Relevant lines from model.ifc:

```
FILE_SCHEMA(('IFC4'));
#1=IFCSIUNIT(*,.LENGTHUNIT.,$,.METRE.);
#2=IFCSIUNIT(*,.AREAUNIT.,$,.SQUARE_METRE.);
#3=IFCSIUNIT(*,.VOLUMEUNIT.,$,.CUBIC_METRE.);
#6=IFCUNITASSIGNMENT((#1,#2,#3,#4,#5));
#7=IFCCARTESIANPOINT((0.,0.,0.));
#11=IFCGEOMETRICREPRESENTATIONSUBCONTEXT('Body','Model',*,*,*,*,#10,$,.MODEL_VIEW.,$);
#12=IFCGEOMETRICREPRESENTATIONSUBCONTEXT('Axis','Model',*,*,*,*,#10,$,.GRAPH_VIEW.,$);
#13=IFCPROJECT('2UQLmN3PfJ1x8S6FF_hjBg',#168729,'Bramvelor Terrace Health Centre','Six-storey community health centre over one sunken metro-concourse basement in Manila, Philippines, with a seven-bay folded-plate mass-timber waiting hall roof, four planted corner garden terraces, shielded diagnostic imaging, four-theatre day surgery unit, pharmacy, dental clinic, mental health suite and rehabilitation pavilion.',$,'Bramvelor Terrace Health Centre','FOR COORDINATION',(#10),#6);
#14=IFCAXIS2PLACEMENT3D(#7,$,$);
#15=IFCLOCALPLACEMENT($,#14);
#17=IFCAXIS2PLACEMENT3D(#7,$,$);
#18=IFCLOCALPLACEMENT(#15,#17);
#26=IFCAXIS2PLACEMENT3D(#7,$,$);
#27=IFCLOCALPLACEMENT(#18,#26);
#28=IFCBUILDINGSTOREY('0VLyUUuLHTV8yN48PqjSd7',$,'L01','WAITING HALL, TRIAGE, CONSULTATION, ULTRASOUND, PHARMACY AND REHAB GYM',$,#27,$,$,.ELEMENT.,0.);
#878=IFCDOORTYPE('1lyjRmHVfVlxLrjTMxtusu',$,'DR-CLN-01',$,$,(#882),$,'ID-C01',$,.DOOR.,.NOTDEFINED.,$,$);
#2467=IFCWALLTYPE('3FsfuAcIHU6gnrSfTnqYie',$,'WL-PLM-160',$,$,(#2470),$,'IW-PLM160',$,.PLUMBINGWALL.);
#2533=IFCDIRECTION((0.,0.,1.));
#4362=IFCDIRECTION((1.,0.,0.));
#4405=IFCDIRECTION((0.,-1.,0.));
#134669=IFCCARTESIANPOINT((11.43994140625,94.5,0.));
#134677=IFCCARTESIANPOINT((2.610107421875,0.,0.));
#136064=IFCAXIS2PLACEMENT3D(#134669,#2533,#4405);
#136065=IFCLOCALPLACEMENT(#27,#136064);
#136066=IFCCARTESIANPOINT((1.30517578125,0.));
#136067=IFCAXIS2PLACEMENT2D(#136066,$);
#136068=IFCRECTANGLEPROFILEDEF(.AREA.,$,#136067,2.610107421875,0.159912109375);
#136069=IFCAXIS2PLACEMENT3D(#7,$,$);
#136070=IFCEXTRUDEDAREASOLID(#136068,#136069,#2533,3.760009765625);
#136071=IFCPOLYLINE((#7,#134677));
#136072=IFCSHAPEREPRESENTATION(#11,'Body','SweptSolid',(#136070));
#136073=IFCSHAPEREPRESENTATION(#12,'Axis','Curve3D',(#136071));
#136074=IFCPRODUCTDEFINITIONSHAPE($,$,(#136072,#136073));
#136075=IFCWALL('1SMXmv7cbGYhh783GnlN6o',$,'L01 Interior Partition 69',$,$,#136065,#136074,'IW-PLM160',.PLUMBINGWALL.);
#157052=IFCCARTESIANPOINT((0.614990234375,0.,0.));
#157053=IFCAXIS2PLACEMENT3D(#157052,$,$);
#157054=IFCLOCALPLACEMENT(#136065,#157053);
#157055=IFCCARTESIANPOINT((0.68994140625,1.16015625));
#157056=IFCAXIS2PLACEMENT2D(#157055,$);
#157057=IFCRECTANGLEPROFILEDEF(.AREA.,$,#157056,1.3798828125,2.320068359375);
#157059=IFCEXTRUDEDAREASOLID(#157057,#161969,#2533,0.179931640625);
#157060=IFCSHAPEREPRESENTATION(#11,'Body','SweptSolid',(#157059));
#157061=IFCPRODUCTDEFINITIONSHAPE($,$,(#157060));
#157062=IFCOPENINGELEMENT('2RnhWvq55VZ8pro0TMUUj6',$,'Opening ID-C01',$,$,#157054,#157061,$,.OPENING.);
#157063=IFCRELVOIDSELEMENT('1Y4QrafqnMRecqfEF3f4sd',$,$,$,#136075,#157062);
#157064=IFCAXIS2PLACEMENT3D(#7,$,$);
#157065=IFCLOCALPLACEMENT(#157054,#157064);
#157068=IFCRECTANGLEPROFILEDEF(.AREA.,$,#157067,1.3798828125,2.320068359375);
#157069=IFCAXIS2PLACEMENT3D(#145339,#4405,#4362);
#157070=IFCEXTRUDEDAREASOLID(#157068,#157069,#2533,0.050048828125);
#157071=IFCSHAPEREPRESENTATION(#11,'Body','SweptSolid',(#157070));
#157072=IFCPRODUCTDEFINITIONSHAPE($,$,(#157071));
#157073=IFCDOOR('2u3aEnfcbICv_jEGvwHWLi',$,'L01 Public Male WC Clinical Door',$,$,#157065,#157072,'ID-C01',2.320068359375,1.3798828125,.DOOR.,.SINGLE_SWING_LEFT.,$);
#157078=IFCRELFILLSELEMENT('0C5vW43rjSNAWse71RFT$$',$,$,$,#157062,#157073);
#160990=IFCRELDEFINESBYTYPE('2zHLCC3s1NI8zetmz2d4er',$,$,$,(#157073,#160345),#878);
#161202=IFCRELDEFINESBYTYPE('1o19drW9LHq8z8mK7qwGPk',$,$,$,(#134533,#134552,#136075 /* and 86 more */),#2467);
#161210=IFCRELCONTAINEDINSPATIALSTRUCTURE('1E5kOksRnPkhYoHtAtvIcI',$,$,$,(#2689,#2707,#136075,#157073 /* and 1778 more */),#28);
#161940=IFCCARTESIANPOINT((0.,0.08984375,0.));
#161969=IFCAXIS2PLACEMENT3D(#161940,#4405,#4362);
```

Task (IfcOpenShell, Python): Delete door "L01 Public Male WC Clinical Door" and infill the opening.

```python
import ifcopenshell
import ifcopenshell.api.feature
import ifcopenshell.api.root
import ifcopenshell.geom
import ifcopenshell.util.shape

model = ifcopenshell.open("model.ifc")
settings = ifcopenshell.geom.settings()


def volume(element):
    """Net volume in cubic metres, openings subtracted."""
    shape = ifcopenshell.geom.create_shape(settings, element)
    return ifcopenshell.util.shape.get_volume(shape.geometry)


door = model.by_guid("2u3aEnfcbICv_jEGvwHWLi")
opening = door.FillsVoids[0].RelatingOpeningElement
wall = opening.VoidsElements[0].RelatingBuildingElement
before = volume(wall)

ifcopenshell.api.root.remove_product(model, product=door)
ifcopenshell.api.feature.remove_feature(model, feature=opening)

after = volume(wall)

print(f"wall volume {before:.3f} -> {after:.3f} m3")

model.write("model_rev.ifc")
```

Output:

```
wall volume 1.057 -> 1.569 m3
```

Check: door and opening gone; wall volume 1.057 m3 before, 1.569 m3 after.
